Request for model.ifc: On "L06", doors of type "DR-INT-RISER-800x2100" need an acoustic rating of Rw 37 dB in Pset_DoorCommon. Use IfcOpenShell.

First a look at what the model holds.

```python
import ifcopenshell
import ifcopenshell.util.element

model = ifcopenshell.open("model.ifc")
print(model.schema)
storey = next(s for s in model.by_type("IfcBuildingStorey") if s.Name == "L06")
doors = [e for e in ifcopenshell.util.element.get_decomposition(storey) if e.is_a("IfcDoor")]
seen = {}
for e in doors:
    element_type = ifcopenshell.util.element.get_type(e)
    key = (element_type.Name if element_type != e and element_type else None, ifcopenshell.util.element.get_pset(e, "Pset_DoorCommon", "AcousticRating"))
    seen[key] = seen.get(key, 0) + 1
for (name, value), count in sorted(seen.items(), key=str):
    print(count, "x", name, "|", value)
```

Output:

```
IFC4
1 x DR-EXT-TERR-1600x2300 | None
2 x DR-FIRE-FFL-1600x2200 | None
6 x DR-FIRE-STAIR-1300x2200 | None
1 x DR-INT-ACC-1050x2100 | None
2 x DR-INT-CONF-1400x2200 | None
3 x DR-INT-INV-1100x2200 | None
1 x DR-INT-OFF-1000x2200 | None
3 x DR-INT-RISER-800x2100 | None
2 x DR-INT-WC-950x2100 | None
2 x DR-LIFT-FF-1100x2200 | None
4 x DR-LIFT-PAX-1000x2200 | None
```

```python
import ifcopenshell
import ifcopenshell.api.pset
import ifcopenshell.util.element

model = ifcopenshell.open("model.ifc")

storey = next(s for s in model.by_type("IfcBuildingStorey") if s.Name == "L06")
doors = [e for e in ifcopenshell.util.element.get_decomposition(storey) if e.is_a("IfcDoor")]

count = 0
for e in doors:
    element_type = ifcopenshell.util.element.get_type(e)
    if element_type in (None, e) or element_type.Name != "DR-INT-RISER-800x2100":
        continue
    # add_pset returns the element's existing set when there is one.
    pset = ifcopenshell.api.pset.add_pset(model, product=e, name="Pset_DoorCommon")
    ifcopenshell.api.pset.edit_pset(model, pset=pset, properties={"AcousticRating": "Rw 37 dB"})
    count += 1

print(count, "doors updated")

model.write("model_v2.ifc")
```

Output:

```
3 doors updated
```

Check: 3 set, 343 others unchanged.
